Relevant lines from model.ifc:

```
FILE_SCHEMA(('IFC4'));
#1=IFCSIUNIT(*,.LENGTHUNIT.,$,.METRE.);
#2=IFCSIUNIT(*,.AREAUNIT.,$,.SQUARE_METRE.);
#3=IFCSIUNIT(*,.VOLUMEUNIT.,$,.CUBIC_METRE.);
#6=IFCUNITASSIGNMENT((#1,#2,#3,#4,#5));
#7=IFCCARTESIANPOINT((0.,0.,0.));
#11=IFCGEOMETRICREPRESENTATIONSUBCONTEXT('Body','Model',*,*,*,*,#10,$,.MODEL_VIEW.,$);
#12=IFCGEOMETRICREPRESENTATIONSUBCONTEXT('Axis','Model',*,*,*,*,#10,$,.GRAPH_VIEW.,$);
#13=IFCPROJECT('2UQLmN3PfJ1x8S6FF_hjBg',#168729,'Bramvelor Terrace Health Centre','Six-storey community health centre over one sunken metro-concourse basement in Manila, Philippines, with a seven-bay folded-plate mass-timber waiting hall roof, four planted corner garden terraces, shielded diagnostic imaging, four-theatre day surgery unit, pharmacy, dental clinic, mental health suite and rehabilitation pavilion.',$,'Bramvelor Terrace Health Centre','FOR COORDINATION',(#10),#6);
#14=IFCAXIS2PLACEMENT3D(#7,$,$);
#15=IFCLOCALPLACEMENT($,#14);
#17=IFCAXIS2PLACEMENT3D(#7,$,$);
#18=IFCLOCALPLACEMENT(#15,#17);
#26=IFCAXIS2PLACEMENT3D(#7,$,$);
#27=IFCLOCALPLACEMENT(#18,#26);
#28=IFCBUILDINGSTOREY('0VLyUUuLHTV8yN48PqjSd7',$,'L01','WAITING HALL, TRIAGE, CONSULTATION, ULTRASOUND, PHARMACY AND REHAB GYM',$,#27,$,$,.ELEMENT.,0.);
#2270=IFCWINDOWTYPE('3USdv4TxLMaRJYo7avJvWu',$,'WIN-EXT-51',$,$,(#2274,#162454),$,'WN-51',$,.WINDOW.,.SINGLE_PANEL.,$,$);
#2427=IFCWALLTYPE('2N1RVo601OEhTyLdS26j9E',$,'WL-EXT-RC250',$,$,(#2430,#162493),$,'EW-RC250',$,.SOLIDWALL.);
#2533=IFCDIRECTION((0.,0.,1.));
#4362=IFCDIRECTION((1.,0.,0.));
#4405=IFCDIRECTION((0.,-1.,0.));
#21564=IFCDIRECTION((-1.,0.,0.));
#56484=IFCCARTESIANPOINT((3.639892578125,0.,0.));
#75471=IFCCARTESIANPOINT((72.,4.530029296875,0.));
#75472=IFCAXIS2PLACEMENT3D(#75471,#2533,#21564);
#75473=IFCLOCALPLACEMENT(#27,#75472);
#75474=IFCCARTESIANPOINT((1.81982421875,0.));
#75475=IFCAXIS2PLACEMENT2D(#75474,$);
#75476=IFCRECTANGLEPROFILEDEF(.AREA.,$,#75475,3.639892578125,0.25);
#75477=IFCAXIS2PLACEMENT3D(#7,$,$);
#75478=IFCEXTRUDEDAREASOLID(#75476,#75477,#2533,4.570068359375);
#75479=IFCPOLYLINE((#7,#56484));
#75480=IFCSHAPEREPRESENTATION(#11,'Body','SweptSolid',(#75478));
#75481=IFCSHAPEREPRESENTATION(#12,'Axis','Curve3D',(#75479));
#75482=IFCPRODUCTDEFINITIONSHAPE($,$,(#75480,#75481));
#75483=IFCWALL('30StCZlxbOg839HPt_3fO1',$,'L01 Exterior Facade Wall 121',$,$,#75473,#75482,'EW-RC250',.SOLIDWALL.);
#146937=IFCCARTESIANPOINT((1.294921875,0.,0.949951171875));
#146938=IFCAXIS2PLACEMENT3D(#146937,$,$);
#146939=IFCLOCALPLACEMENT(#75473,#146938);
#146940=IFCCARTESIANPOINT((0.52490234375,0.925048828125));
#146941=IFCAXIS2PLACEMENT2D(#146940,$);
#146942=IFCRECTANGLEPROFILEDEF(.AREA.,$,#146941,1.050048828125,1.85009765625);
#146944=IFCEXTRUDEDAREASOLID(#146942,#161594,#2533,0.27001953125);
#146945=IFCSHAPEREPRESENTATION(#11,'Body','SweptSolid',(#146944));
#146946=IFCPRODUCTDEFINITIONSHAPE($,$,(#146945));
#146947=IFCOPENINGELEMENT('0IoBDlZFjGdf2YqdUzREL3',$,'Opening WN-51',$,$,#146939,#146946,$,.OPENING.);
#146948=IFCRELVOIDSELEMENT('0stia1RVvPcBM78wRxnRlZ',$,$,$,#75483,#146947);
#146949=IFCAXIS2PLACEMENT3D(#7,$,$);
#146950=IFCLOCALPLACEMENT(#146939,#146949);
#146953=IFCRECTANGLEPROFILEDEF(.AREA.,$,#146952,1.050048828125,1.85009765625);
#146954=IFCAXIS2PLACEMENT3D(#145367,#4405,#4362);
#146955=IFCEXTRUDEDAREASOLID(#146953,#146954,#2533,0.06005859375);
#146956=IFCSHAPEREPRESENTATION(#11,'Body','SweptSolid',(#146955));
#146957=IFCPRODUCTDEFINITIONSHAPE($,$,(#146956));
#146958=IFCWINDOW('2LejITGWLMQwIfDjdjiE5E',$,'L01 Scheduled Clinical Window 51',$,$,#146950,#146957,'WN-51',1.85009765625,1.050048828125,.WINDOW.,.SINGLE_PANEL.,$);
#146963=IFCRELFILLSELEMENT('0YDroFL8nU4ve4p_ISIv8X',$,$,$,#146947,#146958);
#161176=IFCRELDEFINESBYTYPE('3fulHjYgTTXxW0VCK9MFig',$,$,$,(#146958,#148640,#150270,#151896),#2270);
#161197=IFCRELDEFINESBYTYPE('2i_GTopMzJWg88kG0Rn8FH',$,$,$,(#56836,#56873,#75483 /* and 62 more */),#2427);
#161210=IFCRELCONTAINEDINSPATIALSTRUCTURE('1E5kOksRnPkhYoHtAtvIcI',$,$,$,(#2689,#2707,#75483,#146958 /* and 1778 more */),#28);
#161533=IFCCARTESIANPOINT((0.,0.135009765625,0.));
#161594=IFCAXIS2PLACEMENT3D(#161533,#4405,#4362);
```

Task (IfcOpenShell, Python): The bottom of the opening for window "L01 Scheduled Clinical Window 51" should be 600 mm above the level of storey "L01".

```python
import numpy as np
import ifcopenshell
import ifcopenshell.api.geometry
import ifcopenshell.geom
import ifcopenshell.util.element
import ifcopenshell.util.placement
import ifcopenshell.util.shape
import ifcopenshell.util.unit

model = ifcopenshell.open("model.ifc")
unit_scale = ifcopenshell.util.unit.calculate_unit_scale(model)

window = model.by_guid("2LejITGWLMQwIfDjdjiE5E")
opening = window.FillsVoids[0].RelatingOpeningElement
storey = ifcopenshell.util.element.get_container(window, ifc_class="IfcBuildingStorey")
level = ifcopenshell.util.placement.get_local_placement(storey.ObjectPlacement)[2, 3]

# The opening's origin need not be at the sill, so measure its lowest point.
shape = ifcopenshell.geom.create_shape(ifcopenshell.geom.settings(), opening)
bottom = ifcopenshell.util.shape.get_shape_bottom_elevation(shape, shape.geometry) / unit_scale
dz = level + 0.6 / unit_scale - bottom

shift = np.array([0.0, 0.0, dz])
# The window is placed relative to its opening, so it follows when the opening moves.
matrix = ifcopenshell.util.placement.get_local_placement(opening.ObjectPlacement)
matrix[:3, 3] += shift
ifcopenshell.api.geometry.edit_object_placement(
    model, product=opening, matrix=matrix, is_si=False, should_transform_children=True
)

print(f"moved by {dz * unit_scale:+.3f} m")

model.write("model_updated.ifc")
```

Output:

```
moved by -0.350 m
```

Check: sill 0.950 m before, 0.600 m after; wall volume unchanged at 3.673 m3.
